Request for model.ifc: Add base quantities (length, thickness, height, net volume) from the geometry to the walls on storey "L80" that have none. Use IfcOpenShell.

First a look at what the model holds.

```python
import ifcopenshell
import ifcopenshell.util.element
import ifcopenshell.util.unit

model = ifcopenshell.open("model.ifc")
print(model.schema)
for unit_type in ("LENGTHUNIT", "AREAUNIT", "VOLUMEUNIT"):
    print(unit_type, ifcopenshell.util.unit.calculate_unit_scale(model, unit_type))
storey = next(s for s in model.by_type("IfcBuildingStorey") if s.Name == "L80")
walls = [e for e in ifcopenshell.util.element.get_decomposition(storey) if e.is_a("IfcWall")]
for e in sorted(walls, key=lambda e: e.id()):
    print(e.id(), e.is_a(), e.Name, list(ifcopenshell.util.element.get_psets(e, qtos_only=True)), sep=" | ")
```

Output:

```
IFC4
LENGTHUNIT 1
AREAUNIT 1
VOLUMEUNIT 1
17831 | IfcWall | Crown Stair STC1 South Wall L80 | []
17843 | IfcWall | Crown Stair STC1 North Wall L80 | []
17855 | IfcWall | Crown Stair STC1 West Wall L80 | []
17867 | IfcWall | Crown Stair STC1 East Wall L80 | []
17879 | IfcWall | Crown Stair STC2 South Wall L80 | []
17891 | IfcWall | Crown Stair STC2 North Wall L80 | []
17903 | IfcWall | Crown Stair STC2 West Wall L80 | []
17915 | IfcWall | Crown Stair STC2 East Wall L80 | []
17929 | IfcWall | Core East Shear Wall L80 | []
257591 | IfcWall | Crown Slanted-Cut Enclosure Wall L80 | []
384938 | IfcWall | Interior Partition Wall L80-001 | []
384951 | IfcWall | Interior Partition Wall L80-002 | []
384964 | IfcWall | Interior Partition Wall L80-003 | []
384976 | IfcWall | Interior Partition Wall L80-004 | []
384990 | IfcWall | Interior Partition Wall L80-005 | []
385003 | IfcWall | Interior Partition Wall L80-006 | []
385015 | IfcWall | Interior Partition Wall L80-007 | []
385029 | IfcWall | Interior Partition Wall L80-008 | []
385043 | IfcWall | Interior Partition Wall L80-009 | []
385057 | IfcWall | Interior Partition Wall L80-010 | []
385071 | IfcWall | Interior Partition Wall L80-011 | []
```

```python
import ifcopenshell
import ifcopenshell.api.pset
import ifcopenshell.geom
import ifcopenshell.util.element
import ifcopenshell.util.shape
import ifcopenshell.util.unit

model = ifcopenshell.open("model.ifc")
unit_scale = ifcopenshell.util.unit.calculate_unit_scale(model)
volume_scale = ifcopenshell.util.unit.calculate_unit_scale(model, "VOLUMEUNIT")
settings = ifcopenshell.geom.settings()

storey = next(s for s in model.by_type("IfcBuildingStorey") if s.Name == "L80")
walls = [e for e in ifcopenshell.util.element.get_decomposition(storey) if e.is_a("IfcWall")]

for e in sorted(walls, key=lambda e: e.id()):
    if ifcopenshell.util.element.get_psets(e, qtos_only=True, should_inherit=False):
        continue
    # Geometry comes back in metres, in the element's own axes.
    shape = ifcopenshell.geom.create_shape(settings, e)
    values = {
        "Length": ifcopenshell.util.shape.get_x(shape.geometry) / unit_scale,
        "Width": ifcopenshell.util.shape.get_y(shape.geometry) / unit_scale,
        "Height": ifcopenshell.util.shape.get_z(shape.geometry) / unit_scale,
        "NetVolume": ifcopenshell.util.shape.get_volume(shape.geometry) / volume_scale,
    }
    qto = ifcopenshell.api.pset.add_qto(model, product=e, name="Qto_WallBaseQuantities")
    ifcopenshell.api.pset.edit_qto(model, qto=qto, properties=values)
    print(e.id(), {k: round(v, 3) for k, v in values.items()})

model.write("model_edited.ifc")
```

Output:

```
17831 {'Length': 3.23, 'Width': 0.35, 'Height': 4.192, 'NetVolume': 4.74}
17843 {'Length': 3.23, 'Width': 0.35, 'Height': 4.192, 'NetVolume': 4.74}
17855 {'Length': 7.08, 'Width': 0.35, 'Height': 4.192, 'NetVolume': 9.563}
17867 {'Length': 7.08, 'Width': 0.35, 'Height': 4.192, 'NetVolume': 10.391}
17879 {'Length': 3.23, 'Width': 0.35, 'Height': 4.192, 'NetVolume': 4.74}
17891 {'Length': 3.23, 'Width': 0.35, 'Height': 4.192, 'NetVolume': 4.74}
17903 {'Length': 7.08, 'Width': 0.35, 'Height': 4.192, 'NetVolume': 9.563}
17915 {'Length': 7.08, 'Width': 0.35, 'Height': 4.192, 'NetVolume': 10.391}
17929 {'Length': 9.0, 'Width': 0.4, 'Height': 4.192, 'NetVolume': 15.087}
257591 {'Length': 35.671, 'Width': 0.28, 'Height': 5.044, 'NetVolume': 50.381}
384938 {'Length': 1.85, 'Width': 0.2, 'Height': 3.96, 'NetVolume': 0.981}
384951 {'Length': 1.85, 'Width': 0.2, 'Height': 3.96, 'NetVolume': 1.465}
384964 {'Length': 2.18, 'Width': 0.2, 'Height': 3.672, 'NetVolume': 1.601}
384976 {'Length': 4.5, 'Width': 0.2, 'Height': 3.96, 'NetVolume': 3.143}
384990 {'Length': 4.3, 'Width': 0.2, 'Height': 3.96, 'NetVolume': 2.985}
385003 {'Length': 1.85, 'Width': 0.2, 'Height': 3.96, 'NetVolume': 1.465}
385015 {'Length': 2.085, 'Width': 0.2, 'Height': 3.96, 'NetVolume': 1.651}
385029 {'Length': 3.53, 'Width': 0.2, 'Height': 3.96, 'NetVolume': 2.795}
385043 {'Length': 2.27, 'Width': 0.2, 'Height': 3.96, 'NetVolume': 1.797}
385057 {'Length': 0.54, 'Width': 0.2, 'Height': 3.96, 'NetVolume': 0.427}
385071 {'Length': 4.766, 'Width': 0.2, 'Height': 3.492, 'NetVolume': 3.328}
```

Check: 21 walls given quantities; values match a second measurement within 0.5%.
